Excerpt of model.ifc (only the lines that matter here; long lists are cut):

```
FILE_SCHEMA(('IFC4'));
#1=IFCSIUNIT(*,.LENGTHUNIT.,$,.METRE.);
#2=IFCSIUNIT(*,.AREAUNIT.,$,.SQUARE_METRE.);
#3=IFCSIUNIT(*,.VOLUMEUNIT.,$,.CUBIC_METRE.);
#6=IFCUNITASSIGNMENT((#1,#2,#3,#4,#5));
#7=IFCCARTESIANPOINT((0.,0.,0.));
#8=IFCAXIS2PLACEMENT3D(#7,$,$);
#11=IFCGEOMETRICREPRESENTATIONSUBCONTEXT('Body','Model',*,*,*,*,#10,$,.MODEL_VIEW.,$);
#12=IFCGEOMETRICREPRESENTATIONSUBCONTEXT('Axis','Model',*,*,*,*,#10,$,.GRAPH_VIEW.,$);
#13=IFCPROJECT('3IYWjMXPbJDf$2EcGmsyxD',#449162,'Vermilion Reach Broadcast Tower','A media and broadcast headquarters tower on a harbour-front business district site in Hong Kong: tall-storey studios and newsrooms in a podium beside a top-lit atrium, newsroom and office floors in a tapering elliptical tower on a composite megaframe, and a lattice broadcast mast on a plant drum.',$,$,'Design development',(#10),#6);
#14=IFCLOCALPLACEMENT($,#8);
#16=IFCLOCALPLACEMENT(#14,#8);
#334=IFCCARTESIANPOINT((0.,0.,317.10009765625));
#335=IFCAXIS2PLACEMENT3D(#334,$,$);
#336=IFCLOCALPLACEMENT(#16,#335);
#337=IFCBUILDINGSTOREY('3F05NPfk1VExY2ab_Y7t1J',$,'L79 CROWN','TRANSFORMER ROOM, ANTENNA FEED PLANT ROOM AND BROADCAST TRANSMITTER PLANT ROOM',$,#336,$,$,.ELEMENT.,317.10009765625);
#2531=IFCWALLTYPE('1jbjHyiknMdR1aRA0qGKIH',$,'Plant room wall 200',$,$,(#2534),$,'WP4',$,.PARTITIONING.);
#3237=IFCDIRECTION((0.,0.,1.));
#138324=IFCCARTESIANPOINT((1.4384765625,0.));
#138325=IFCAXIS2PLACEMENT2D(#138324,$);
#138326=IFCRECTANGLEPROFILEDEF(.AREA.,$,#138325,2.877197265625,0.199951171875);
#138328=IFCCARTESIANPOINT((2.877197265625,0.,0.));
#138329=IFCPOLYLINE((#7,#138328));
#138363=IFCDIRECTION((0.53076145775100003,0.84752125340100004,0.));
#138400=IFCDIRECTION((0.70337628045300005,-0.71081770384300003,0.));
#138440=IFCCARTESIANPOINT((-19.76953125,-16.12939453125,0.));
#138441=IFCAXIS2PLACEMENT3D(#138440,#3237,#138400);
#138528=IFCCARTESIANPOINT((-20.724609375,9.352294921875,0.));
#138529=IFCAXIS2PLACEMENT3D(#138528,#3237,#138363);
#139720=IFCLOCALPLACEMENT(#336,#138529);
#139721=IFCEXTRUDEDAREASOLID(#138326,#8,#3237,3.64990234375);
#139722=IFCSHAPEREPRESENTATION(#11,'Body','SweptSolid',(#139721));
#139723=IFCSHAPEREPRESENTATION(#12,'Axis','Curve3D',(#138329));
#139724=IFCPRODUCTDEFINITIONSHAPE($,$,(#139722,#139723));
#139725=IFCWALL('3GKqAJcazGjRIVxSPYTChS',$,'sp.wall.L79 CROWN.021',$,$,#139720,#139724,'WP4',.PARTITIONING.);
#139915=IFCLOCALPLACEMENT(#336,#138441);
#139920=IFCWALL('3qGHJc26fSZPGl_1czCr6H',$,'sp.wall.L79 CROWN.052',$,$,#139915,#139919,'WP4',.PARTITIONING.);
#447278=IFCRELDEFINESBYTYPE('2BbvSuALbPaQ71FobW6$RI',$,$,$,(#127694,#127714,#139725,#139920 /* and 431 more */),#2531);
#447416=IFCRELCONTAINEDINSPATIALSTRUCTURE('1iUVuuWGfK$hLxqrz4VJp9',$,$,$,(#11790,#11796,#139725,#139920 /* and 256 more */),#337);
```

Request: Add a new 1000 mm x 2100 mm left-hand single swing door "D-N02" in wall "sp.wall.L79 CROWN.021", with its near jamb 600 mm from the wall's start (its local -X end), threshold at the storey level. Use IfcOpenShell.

```python
import numpy as np
import ifcopenshell
import ifcopenshell.api.feature
import ifcopenshell.api.geometry
import ifcopenshell.api.root
import ifcopenshell.api.spatial
import ifcopenshell.geom
import ifcopenshell.util.element
import ifcopenshell.util.placement
import ifcopenshell.util.representation
import ifcopenshell.util.shape
import ifcopenshell.util.unit

model = ifcopenshell.open("model.ifc")
unit_scale = ifcopenshell.util.unit.calculate_unit_scale(model)
settings = ifcopenshell.geom.settings()


def volume(element):
    """Net volume in cubic metres, openings subtracted."""
    shape = ifcopenshell.geom.create_shape(settings, element)
    return ifcopenshell.util.shape.get_volume(shape.geometry)


wall = model.by_id(139725)
storey = ifcopenshell.util.element.get_container(wall, ifc_class="IfcBuildingStorey")
context = ifcopenshell.util.representation.get_context(model, "Model", "Body", "MODEL_VIEW")
before = volume(wall)

width, height, from_end, sill = 1, 2.1, 0.6, 0.0  # metres

# The wall runs along its own X axis, and the end named is its -X end.
wall_shape = ifcopenshell.geom.create_shape(settings, wall)
x, y, z = ifcopenshell.util.shape.get_vertices(wall_shape.geometry).T
start = x.min() + from_end
face, thickness = float(y.min()), float(y.max() - y.min())
wall_matrix = ifcopenshell.util.placement.get_local_placement(wall.ObjectPlacement)
level = ifcopenshell.util.placement.get_local_placement(storey.ObjectPlacement)[2, 3]


def in_wall(x, y):
    """Placement at x, y metres in the wall's axes, at sill height."""
    matrix = wall_matrix.copy()
    matrix[:, 3] = wall_matrix @ np.array([x / unit_scale, y / unit_scale, 0.0, 1.0])
    matrix[2, 3] = level + sill / unit_scale
    return matrix


# Opening: a box that overshoots both wall faces by 50 mm.
opening = ifcopenshell.api.root.create_entity(model, ifc_class="IfcOpeningElement", predefined_type="OPENING")
box = ifcopenshell.api.geometry.add_wall_representation(
    model, context=context, length=width, height=height, thickness=thickness + 0.1
)
ifcopenshell.api.geometry.assign_representation(model, product=opening, representation=box)
ifcopenshell.api.geometry.edit_object_placement(model, product=opening, matrix=in_wall(start, face - 0.05), is_si=False)
ifcopenshell.api.feature.add_feature(model, feature=opening, element=wall)

door = ifcopenshell.api.root.create_entity(model, ifc_class="IfcDoor", name="D-N02", predefined_type="DOOR")
door.OverallWidth, door.OverallHeight = width / unit_scale, height / unit_scale
door.OperationType = "SINGLE_SWING_LEFT"
body = ifcopenshell.api.geometry.add_door_representation(
    model,
    context=context,
    overall_width=door.OverallWidth,
    overall_height=door.OverallHeight,
    operation_type="SINGLE_SWING_LEFT",
    lining_properties={"LiningDepth": thickness / unit_scale, "ThresholdDepth": thickness / unit_scale},
)
ifcopenshell.api.geometry.assign_representation(model, product=door, representation=body)
ifcopenshell.api.spatial.assign_container(model, products=[door], relating_structure=storey)
ifcopenshell.api.feature.add_filling(model, opening=opening, element=door)

# The lining spans the wall, so the door starts at the wall face.
ifcopenshell.api.geometry.edit_object_placement(model, product=door, matrix=in_wall(start, face), is_si=False)

after = volume(wall)

print(f"wall volume {before:.3f} -> {after:.3f} m3")

model.write("model_edited.ifc")
```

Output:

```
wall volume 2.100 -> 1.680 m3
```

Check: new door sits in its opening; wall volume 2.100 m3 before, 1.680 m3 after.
